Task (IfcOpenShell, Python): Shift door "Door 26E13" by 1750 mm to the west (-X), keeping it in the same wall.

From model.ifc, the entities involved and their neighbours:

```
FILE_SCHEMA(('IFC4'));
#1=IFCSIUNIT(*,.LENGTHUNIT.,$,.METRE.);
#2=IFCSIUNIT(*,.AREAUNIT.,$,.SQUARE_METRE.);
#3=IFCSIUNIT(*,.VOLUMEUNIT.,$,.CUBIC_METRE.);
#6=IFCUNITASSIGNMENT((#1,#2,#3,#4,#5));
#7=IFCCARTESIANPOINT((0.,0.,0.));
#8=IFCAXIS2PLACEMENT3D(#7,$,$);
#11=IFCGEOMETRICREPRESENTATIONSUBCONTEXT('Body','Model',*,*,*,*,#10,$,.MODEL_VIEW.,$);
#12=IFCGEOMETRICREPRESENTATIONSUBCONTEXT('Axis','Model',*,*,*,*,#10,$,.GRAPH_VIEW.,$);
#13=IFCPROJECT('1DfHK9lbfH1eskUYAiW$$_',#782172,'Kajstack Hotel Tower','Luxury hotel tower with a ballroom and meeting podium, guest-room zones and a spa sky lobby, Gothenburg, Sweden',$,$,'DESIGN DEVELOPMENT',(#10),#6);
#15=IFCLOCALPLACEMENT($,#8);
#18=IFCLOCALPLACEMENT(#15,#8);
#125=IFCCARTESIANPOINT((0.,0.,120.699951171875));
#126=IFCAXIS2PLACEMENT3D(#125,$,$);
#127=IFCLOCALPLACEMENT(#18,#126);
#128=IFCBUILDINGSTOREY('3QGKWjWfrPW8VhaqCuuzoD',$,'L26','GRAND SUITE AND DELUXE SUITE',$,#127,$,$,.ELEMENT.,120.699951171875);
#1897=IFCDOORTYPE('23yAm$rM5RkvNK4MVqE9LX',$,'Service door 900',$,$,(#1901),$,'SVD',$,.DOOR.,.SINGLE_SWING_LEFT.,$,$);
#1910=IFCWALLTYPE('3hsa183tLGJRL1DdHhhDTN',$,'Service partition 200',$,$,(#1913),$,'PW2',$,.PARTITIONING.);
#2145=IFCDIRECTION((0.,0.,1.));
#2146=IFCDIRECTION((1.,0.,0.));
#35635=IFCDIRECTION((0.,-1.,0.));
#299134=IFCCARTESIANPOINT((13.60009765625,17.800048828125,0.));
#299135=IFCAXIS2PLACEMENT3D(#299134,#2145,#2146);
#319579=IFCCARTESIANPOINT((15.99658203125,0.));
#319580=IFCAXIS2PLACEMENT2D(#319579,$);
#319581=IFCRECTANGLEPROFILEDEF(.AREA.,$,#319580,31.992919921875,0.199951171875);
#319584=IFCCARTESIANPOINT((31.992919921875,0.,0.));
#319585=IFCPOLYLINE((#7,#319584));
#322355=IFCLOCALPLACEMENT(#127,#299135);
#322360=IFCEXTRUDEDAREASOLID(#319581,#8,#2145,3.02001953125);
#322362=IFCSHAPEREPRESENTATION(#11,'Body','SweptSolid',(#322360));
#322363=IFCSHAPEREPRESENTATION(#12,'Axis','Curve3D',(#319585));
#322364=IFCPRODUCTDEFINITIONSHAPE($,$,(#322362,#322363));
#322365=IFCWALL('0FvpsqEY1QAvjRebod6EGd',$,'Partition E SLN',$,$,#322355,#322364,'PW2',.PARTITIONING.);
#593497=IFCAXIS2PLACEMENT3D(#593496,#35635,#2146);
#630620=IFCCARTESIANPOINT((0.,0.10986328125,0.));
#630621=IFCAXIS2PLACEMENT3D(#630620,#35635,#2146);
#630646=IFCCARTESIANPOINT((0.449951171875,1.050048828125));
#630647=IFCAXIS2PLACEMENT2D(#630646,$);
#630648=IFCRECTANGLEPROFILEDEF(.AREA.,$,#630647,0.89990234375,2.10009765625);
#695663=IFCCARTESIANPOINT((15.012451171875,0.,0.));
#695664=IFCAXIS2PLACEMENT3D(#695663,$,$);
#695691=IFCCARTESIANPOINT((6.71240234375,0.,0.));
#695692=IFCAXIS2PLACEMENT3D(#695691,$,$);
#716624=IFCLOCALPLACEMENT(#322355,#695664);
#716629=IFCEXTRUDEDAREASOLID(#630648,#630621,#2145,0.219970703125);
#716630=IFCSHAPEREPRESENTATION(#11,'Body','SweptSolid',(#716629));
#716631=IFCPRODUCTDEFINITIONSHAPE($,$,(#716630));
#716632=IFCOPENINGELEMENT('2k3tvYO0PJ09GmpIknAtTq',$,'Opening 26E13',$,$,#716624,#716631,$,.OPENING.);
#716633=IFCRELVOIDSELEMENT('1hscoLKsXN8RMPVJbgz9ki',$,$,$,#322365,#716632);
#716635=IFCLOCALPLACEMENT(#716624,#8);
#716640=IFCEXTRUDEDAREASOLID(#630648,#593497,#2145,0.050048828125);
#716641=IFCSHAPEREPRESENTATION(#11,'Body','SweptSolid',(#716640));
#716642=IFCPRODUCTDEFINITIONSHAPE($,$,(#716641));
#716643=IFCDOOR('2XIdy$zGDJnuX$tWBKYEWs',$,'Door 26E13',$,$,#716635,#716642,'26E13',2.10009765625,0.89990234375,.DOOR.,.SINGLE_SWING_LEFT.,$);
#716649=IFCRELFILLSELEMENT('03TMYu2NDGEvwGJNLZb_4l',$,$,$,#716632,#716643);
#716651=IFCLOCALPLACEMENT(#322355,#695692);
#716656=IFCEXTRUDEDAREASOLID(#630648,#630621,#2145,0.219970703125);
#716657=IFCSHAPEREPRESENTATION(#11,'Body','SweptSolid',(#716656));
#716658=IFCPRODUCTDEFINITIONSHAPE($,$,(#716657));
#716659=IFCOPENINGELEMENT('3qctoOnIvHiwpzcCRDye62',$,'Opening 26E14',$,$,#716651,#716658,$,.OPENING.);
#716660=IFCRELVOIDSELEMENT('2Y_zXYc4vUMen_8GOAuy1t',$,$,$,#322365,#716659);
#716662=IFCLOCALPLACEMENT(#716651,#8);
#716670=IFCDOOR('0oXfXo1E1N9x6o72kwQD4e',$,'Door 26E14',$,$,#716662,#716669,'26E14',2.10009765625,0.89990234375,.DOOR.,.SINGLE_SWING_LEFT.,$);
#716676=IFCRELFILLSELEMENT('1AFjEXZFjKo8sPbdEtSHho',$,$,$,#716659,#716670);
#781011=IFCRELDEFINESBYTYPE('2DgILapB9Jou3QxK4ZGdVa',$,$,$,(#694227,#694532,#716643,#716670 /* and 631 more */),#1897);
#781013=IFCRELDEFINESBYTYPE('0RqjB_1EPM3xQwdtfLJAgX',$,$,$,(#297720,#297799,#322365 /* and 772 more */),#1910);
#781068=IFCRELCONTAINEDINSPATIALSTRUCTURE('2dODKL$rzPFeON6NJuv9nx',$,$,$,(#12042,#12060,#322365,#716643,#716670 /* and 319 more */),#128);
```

```python
import ifcopenshell
import ifcopenshell.api.geometry
import ifcopenshell.util.placement
import ifcopenshell.util.unit

model = ifcopenshell.open("model.ifc")
unit_scale = ifcopenshell.util.unit.calculate_unit_scale(model)

door = model.by_guid("2XIdy$zGDJnuX$tWBKYEWs")
opening = door.FillsVoids[0].RelatingOpeningElement
wall = opening.VoidsElements[0].RelatingBuildingElement

wall_matrix = ifcopenshell.util.placement.get_local_placement(wall.ObjectPlacement)
shift = wall_matrix[:3, 0] * -1.75 / unit_scale
before = ifcopenshell.util.placement.get_local_placement(door.ObjectPlacement)[:3, 3].copy()

# The door is placed relative to its opening, so it follows when the opening moves.
matrix = ifcopenshell.util.placement.get_local_placement(opening.ObjectPlacement)
matrix[:3, 3] += shift
ifcopenshell.api.geometry.edit_object_placement(
    model, product=opening, matrix=matrix, is_si=False, should_transform_children=True
)

after = ifcopenshell.util.placement.get_local_placement(door.ObjectPlacement)[:3, 3]
print("door moved by", (after - before).round(3) + 0.0)

model.write("model_rev.ifc")
```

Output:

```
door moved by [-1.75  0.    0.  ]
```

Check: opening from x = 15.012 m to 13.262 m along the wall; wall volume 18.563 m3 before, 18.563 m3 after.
